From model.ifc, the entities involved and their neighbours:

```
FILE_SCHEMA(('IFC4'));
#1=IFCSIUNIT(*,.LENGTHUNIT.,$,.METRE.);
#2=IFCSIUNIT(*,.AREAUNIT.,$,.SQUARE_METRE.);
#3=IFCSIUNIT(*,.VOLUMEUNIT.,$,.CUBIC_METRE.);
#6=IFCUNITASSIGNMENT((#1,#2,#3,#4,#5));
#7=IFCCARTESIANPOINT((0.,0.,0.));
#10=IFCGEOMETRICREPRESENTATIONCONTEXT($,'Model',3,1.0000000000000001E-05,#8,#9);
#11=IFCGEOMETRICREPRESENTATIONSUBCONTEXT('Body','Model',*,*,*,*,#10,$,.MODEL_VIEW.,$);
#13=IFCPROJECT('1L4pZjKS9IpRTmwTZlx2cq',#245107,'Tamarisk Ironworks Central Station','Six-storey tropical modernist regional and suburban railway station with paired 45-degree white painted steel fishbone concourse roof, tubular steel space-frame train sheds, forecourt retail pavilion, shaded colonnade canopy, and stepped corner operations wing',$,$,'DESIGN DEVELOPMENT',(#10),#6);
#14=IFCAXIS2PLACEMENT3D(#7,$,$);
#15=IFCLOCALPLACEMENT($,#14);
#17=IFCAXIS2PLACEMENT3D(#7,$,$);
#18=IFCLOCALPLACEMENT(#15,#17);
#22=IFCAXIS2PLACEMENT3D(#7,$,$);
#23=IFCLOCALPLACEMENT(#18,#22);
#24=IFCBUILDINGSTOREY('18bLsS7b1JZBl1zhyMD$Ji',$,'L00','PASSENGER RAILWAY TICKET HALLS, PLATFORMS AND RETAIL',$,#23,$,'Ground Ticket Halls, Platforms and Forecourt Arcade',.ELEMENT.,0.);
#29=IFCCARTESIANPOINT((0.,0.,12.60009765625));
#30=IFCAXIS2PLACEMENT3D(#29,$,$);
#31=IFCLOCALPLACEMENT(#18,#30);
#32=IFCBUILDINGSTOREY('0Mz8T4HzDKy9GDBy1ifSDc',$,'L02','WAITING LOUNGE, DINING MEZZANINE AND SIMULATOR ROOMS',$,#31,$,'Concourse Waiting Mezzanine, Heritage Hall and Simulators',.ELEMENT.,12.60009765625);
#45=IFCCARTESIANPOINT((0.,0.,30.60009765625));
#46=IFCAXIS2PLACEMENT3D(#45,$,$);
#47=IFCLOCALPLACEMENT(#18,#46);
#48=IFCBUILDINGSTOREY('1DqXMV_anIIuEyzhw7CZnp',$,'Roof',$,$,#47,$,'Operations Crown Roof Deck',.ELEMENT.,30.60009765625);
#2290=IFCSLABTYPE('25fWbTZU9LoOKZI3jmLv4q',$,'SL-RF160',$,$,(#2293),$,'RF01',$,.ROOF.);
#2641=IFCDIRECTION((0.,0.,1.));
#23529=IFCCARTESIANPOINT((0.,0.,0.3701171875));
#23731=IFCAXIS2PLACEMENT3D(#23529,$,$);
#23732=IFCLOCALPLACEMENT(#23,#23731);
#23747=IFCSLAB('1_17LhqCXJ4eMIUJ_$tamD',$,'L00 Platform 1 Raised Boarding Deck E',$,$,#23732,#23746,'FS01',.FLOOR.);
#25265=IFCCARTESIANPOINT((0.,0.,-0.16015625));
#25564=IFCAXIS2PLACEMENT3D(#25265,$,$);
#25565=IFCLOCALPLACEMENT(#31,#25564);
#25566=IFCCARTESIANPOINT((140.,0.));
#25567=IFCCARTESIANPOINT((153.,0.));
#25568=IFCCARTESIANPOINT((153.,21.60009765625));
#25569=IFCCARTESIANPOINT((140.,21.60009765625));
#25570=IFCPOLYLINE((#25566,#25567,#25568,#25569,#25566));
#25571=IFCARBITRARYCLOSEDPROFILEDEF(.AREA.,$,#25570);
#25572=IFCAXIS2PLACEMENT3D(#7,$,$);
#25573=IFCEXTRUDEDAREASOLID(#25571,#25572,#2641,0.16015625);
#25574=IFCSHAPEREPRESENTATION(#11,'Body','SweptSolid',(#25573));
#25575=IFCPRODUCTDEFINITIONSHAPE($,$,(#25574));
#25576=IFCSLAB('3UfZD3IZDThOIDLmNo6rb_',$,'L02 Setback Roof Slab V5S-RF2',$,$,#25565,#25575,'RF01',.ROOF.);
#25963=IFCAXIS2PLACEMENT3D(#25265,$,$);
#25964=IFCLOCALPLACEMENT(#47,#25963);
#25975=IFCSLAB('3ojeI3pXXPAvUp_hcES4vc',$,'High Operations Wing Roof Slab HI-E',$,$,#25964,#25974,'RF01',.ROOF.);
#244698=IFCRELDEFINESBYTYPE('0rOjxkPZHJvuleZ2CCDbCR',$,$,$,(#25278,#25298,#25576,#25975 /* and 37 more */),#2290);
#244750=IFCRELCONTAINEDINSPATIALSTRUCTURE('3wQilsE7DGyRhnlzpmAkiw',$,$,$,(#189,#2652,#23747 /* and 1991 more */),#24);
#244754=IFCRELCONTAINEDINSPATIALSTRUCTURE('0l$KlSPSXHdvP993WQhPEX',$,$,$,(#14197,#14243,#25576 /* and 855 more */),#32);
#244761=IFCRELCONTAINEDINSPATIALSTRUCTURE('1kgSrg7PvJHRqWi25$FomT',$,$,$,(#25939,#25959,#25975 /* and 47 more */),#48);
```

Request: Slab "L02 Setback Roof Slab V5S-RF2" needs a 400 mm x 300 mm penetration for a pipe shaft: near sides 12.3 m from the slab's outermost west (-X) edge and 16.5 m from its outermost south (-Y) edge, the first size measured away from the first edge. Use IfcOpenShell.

```python
import numpy as np
import ifcopenshell
import ifcopenshell.api.feature
import ifcopenshell.api.geometry
import ifcopenshell.api.root
import ifcopenshell.geom
import ifcopenshell.util.placement
import ifcopenshell.util.representation
import ifcopenshell.util.shape
import ifcopenshell.util.unit

model = ifcopenshell.open("model.ifc")
unit_scale = ifcopenshell.util.unit.calculate_unit_scale(model)
settings = ifcopenshell.geom.settings()


def volume(element):
    """Net volume in cubic metres, openings subtracted."""
    shape = ifcopenshell.geom.create_shape(settings, element)
    return ifcopenshell.util.shape.get_volume(shape.geometry)


slab = model.by_guid("3UfZD3IZDThOIDLmNo6rb_")
before = volume(slab)

# Extent in the slab's own axes, in metres. The edges named are its -X and -Y sides.
slab_shape = ifcopenshell.geom.create_shape(settings, slab)
vertices = ifcopenshell.util.shape.get_vertices(slab_shape.geometry)
x_min, y_min, bottom = vertices.min(axis=0)
top = vertices[:, 2].max()

opening = ifcopenshell.api.root.create_entity(model, ifc_class="IfcOpeningElement", name="Pipe shaft opening", predefined_type="OPENING")
context = ifcopenshell.util.representation.get_context(model, "Model", "Body", "MODEL_VIEW")
width, depth = 0.4, 0.3
outline = [(0.0, 0.0), (width, 0.0), (width, depth), (0.0, depth), (0.0, 0.0)]
# Overshoot both faces by 50 mm so the cut is clean.
shape = ifcopenshell.api.geometry.add_slab_representation(
    model, context=context, depth=top - bottom + 0.1, polyline=outline
)
ifcopenshell.api.geometry.assign_representation(model, product=opening, representation=shape)

matrix = ifcopenshell.util.placement.get_local_placement(slab.ObjectPlacement)
matrix[:, 3] = matrix @ np.append(np.array([x_min + 12.3, y_min + 16.5, bottom - 0.05]) / unit_scale, 1.0)
ifcopenshell.api.geometry.edit_object_placement(model, product=opening, matrix=matrix, is_si=False)
ifcopenshell.api.feature.add_feature(model, feature=opening, element=slab)

after = volume(slab)

print(f"slab volume {before:.3f} -> {after:.3f} m3")

model.write("model_updated.ifc")
```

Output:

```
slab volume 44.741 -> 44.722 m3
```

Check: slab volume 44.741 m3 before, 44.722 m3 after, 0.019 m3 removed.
